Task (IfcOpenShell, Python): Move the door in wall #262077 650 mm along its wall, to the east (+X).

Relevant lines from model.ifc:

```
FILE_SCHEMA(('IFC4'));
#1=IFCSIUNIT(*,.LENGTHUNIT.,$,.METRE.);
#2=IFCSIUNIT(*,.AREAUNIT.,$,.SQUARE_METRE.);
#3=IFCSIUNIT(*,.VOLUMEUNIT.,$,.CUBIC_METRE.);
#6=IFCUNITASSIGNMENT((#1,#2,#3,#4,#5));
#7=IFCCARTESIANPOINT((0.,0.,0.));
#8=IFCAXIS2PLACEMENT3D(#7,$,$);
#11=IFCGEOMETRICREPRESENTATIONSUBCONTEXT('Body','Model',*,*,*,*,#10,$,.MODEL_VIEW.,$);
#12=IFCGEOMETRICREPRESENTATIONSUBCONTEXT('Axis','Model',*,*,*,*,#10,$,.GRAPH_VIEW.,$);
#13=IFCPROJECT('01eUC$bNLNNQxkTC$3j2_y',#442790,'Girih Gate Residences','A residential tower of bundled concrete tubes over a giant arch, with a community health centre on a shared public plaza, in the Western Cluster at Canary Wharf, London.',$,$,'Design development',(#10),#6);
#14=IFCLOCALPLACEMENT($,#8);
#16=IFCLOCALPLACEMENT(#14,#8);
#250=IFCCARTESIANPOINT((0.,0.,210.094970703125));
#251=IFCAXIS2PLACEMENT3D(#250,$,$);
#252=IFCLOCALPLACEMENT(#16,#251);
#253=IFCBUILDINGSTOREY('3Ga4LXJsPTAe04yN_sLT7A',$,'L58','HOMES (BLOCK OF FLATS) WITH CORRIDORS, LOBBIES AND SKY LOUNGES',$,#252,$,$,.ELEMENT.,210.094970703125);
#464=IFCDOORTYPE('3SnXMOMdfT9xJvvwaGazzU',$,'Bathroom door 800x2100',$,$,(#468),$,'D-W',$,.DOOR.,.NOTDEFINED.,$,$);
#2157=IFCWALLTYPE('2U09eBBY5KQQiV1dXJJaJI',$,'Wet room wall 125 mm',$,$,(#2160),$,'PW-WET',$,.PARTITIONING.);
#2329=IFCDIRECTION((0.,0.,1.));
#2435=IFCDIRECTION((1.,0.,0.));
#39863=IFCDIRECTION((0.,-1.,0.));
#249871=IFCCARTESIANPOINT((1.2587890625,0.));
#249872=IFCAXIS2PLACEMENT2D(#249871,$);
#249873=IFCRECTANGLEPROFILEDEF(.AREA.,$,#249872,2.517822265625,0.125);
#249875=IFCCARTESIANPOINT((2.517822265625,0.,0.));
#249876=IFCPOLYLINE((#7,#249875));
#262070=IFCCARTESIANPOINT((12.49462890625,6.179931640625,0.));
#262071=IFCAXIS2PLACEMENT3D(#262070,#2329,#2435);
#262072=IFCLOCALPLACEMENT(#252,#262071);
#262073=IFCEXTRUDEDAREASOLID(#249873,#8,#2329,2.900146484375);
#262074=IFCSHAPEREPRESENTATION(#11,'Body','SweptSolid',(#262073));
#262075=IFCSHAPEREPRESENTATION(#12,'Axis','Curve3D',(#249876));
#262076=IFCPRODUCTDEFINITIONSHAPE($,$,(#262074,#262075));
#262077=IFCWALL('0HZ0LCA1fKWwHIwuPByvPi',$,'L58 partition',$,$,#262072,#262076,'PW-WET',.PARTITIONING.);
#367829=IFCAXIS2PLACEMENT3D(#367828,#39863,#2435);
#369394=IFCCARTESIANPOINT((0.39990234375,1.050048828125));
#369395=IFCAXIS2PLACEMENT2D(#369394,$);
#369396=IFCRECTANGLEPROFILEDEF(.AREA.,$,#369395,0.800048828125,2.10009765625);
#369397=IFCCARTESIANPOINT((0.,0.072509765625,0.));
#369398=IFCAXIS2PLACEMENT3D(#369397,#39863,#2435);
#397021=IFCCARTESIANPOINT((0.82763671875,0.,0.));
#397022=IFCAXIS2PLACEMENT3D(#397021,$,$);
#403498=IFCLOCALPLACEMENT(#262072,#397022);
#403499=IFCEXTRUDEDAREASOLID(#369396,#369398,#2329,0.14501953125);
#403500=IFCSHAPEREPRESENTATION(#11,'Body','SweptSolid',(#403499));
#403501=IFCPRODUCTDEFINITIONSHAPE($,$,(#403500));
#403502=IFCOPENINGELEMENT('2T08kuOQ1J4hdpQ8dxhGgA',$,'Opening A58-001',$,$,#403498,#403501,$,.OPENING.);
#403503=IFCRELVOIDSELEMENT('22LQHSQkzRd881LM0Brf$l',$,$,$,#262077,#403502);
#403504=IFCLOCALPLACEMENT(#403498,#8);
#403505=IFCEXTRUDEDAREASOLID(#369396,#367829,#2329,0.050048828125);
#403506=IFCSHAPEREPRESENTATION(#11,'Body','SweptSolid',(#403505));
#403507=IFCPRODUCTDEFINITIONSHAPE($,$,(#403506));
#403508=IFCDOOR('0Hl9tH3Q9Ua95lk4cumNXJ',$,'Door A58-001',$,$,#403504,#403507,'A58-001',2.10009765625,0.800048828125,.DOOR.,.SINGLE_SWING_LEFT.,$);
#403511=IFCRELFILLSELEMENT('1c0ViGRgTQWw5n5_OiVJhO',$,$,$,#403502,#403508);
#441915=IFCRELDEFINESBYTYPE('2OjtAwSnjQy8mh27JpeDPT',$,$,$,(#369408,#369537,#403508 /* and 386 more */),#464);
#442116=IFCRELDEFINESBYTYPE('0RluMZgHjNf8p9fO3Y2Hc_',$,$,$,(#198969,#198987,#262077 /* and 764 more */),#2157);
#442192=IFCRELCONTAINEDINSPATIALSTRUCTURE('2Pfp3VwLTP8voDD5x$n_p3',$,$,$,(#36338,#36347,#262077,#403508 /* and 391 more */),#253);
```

```python
import ifcopenshell
import ifcopenshell.api.geometry
import ifcopenshell.util.placement
import ifcopenshell.util.unit

model = ifcopenshell.open("model.ifc")
unit_scale = ifcopenshell.util.unit.calculate_unit_scale(model)

door = model.by_guid("0Hl9tH3Q9Ua95lk4cumNXJ")
opening = door.FillsVoids[0].RelatingOpeningElement
wall = opening.VoidsElements[0].RelatingBuildingElement

wall_matrix = ifcopenshell.util.placement.get_local_placement(wall.ObjectPlacement)
shift = wall_matrix[:3, 0] * 0.65 / unit_scale
before = ifcopenshell.util.placement.get_local_placement(door.ObjectPlacement)[:3, 3].copy()

# The door is placed relative to its opening, so it follows when the opening moves.
matrix = ifcopenshell.util.placement.get_local_placement(opening.ObjectPlacement)
matrix[:3, 3] += shift
ifcopenshell.api.geometry.edit_object_placement(
    model, product=opening, matrix=matrix, is_si=False, should_transform_children=True
)

after = ifcopenshell.util.placement.get_local_placement(door.ObjectPlacement)[:3, 3]
print("door moved by", (after - before).round(3) + 0.0)

model.write("model_updated.ifc")
```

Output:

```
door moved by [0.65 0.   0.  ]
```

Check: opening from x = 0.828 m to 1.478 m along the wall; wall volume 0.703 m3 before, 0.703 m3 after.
